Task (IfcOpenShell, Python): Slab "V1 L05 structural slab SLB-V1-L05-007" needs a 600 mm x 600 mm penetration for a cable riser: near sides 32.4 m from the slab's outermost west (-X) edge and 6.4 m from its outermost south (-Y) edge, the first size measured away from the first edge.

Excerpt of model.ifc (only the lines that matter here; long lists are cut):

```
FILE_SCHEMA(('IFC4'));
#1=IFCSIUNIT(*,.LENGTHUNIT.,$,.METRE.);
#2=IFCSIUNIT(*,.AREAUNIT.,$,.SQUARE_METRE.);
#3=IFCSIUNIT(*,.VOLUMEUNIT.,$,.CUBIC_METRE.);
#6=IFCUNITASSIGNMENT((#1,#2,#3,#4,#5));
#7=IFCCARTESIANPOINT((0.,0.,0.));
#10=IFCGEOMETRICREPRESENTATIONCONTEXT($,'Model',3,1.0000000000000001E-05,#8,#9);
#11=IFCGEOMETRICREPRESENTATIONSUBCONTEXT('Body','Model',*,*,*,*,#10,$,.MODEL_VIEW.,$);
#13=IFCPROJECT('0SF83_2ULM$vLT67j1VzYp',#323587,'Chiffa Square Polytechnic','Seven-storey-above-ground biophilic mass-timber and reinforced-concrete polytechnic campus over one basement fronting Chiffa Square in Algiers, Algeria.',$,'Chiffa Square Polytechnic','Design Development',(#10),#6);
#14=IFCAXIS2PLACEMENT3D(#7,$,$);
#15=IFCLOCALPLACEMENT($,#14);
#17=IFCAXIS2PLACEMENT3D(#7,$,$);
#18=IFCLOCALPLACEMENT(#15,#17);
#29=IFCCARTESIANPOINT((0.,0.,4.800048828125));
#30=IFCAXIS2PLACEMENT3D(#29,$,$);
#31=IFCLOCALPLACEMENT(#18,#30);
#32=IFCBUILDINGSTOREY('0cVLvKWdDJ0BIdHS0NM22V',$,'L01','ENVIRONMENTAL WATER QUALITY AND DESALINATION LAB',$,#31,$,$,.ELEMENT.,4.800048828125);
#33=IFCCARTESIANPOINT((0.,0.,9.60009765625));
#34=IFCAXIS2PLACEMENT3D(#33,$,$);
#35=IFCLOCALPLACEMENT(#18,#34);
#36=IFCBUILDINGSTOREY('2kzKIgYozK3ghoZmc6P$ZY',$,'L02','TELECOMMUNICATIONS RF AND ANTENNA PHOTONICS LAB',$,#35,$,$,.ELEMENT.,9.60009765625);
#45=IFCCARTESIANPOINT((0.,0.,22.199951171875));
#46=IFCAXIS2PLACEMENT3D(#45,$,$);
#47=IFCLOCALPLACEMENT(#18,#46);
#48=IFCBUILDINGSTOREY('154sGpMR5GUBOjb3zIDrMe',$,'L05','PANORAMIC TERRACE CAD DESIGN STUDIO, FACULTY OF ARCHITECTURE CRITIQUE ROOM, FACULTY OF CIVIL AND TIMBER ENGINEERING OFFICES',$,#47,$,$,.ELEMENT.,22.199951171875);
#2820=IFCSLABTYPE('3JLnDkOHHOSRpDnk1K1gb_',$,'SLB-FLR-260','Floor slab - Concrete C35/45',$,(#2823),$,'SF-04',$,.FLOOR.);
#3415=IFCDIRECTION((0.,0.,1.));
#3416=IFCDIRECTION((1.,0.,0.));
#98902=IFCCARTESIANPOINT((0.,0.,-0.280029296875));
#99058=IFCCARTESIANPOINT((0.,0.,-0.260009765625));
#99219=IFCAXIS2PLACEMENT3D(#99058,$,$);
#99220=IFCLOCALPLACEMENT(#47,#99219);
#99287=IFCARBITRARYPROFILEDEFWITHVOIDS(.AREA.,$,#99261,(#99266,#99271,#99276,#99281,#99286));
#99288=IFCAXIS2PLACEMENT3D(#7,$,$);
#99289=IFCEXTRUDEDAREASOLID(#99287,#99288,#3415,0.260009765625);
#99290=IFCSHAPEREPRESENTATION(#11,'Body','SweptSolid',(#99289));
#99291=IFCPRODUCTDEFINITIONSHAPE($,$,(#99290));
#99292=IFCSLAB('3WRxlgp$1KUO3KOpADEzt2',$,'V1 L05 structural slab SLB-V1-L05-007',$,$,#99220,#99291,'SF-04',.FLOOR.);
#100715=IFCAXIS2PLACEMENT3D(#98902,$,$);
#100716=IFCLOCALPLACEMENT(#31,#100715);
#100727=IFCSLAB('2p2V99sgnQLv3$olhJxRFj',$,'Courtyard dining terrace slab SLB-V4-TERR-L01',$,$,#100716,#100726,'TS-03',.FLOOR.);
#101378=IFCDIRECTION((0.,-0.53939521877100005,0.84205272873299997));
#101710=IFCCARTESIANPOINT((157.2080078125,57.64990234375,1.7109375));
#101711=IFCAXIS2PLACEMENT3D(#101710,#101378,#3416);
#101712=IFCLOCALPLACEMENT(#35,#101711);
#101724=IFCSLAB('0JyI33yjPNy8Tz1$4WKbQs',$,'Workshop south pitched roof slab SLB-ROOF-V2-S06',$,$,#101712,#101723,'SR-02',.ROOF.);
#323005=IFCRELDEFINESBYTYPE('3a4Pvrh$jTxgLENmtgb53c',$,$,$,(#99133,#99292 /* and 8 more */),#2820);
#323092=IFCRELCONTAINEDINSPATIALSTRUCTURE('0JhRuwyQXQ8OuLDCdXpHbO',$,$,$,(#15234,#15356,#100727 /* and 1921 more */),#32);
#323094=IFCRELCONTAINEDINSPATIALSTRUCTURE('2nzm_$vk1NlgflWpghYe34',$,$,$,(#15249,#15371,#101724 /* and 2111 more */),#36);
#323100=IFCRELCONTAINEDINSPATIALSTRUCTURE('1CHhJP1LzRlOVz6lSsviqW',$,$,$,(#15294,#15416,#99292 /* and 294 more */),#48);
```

```python
import numpy as np
import ifcopenshell
import ifcopenshell.api.feature
import ifcopenshell.api.geometry
import ifcopenshell.api.root
import ifcopenshell.geom
import ifcopenshell.util.placement
import ifcopenshell.util.representation
import ifcopenshell.util.shape
import ifcopenshell.util.unit

model = ifcopenshell.open("model.ifc")
unit_scale = ifcopenshell.util.unit.calculate_unit_scale(model)
settings = ifcopenshell.geom.settings()


def volume(element):
    """Net volume in cubic metres, openings subtracted."""
    shape = ifcopenshell.geom.create_shape(settings, element)
    return ifcopenshell.util.shape.get_volume(shape.geometry)


slab = model.by_id(99292)
before = volume(slab)

# Extent in the slab's own axes, in metres. The edges named are its -X and -Y sides.
slab_shape = ifcopenshell.geom.create_shape(settings, slab)
vertices = ifcopenshell.util.shape.get_vertices(slab_shape.geometry)
x_min, y_min, bottom = vertices.min(axis=0)
top = vertices[:, 2].max()

opening = ifcopenshell.api.root.create_entity(model, ifc_class="IfcOpeningElement", name="Cable riser opening", predefined_type="OPENING")
context = ifcopenshell.util.representation.get_context(model, "Model", "Body", "MODEL_VIEW")
width, depth = 0.6, 0.6
outline = [(0.0, 0.0), (width, 0.0), (width, depth), (0.0, depth), (0.0, 0.0)]
# Overshoot both faces by 50 mm so the cut is clean.
shape = ifcopenshell.api.geometry.add_slab_representation(
    model, context=context, depth=top - bottom + 0.1, polyline=outline
)
ifcopenshell.api.geometry.assign_representation(model, product=opening, representation=shape)

matrix = ifcopenshell.util.placement.get_local_placement(slab.ObjectPlacement)
matrix[:, 3] = matrix @ np.append(np.array([x_min + 32.4, y_min + 6.4, bottom - 0.05]) / unit_scale, 1.0)
ifcopenshell.api.geometry.edit_object_placement(model, product=opening, matrix=matrix, is_si=False)
ifcopenshell.api.feature.add_feature(model, feature=opening, element=slab)

after = volume(slab)

print(f"slab volume {before:.3f} -> {after:.3f} m3")

model.write("model-out.ifc")
```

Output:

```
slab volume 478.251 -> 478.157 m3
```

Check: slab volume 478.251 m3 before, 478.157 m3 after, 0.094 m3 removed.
